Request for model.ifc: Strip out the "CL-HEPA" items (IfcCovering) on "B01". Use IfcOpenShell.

First a look at what the model holds.

```python
import ifcopenshell
import ifcopenshell.util.element

model = ifcopenshell.open("model.ifc")
print(model.schema)
storey = next(s for s in model.by_type("IfcBuildingStorey") if s.Name == "B01")
coverings = [e for e in ifcopenshell.util.element.get_decomposition(storey) if e.is_a("IfcCovering")]
seen = {}
for e in coverings:
    element_type = ifcopenshell.util.element.get_type(e)
    name = element_type.Name if element_type not in (None, e) else None
    seen[name] = seen.get(name, 0) + 1
for name, count in sorted(seen.items(), key=str):
    print(count, "x", name)
```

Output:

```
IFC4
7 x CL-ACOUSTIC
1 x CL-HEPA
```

```python
import ifcopenshell
import ifcopenshell.api.root
import ifcopenshell.util.element

model = ifcopenshell.open("model.ifc")

storey = next(s for s in model.by_type("IfcBuildingStorey") if s.Name == "B01")
coverings = [e for e in ifcopenshell.util.element.get_decomposition(storey) if e.is_a("IfcCovering")]
targets = [e for e in coverings if (t := ifcopenshell.util.element.get_type(e)) not in (None, e) and t.Name == "CL-HEPA"]

for e in targets:
    ifcopenshell.api.root.remove_product(model, product=e)
print(len(targets), "removed")

model.write("model_edited.ifc")
```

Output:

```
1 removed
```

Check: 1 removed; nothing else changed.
